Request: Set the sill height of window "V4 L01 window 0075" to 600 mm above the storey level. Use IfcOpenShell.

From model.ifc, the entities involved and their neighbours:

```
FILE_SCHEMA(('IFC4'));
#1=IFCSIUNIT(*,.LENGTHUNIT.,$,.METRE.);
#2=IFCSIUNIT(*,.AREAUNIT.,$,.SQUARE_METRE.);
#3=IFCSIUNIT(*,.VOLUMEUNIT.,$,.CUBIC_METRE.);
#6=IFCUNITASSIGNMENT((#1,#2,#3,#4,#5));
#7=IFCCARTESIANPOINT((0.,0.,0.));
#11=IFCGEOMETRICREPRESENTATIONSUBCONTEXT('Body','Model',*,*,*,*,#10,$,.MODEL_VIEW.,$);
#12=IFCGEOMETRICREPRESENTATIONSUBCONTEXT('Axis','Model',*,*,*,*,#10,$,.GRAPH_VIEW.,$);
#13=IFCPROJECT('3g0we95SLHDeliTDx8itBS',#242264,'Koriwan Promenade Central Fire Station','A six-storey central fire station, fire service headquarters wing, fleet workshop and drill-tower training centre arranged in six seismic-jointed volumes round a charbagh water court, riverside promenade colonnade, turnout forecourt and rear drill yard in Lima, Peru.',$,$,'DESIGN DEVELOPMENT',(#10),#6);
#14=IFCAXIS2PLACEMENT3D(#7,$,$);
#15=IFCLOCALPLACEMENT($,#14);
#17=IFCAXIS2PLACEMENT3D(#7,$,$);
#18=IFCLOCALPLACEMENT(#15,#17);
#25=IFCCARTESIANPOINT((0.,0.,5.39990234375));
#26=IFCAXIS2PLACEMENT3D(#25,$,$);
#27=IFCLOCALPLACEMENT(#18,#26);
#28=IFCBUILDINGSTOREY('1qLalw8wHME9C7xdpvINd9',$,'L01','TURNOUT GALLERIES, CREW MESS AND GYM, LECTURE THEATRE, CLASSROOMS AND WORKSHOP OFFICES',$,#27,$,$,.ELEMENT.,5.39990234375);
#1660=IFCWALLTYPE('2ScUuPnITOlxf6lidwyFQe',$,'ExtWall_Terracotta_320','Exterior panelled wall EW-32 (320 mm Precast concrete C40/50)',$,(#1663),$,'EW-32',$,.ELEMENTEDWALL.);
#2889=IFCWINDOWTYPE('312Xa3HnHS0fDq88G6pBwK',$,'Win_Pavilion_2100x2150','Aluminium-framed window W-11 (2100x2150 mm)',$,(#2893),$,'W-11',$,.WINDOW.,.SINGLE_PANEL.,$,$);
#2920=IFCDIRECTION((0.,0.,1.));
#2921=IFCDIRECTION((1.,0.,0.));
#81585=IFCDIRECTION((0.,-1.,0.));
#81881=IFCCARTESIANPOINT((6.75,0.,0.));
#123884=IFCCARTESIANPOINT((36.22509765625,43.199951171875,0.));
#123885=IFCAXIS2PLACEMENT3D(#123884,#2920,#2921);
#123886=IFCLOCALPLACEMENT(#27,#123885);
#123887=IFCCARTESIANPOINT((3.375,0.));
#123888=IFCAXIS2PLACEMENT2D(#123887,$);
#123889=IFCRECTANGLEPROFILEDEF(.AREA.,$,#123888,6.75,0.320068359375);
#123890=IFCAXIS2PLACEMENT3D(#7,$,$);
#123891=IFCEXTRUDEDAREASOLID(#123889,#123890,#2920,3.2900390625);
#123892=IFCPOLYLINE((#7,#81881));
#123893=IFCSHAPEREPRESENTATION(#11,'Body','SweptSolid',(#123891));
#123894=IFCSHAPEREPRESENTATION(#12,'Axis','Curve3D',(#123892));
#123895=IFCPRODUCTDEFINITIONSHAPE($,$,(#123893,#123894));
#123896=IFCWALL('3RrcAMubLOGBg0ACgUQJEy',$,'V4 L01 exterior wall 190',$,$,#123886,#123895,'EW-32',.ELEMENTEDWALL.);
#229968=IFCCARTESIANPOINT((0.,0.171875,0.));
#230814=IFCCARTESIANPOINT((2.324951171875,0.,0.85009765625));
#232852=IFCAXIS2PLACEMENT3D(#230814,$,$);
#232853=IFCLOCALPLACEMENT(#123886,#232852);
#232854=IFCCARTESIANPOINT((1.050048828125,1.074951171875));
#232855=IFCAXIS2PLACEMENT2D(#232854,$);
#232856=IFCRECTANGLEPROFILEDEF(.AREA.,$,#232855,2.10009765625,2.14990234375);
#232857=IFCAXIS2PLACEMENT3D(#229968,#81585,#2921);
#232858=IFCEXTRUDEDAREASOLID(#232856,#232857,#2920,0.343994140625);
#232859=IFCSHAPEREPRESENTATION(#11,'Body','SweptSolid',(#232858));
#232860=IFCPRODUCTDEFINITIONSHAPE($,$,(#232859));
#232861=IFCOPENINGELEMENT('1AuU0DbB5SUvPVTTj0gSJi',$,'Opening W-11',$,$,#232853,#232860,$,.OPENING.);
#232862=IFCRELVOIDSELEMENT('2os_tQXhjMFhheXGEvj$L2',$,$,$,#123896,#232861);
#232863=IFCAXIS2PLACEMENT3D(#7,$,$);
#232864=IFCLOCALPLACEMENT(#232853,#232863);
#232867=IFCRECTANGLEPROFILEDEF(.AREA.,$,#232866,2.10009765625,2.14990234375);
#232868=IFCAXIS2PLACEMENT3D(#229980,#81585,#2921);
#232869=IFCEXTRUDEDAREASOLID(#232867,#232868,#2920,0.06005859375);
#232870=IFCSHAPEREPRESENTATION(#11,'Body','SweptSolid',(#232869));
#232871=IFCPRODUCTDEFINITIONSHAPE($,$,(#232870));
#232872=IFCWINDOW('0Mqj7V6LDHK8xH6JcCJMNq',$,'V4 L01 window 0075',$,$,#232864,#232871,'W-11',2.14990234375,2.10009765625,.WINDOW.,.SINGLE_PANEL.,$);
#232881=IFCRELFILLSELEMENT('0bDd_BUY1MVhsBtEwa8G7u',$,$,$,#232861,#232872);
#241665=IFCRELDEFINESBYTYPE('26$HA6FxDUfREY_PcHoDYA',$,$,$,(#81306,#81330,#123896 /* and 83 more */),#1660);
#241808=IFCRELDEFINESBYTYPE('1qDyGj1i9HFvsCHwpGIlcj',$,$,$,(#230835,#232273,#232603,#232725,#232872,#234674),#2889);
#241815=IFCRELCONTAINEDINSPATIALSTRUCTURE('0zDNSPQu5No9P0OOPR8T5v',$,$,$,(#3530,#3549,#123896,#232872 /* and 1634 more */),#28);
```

```python
import numpy as np
import ifcopenshell
import ifcopenshell.api.geometry
import ifcopenshell.geom
import ifcopenshell.util.element
import ifcopenshell.util.placement
import ifcopenshell.util.shape
import ifcopenshell.util.unit

model = ifcopenshell.open("model.ifc")
unit_scale = ifcopenshell.util.unit.calculate_unit_scale(model)

window = model.by_guid("0Mqj7V6LDHK8xH6JcCJMNq")
opening = window.FillsVoids[0].RelatingOpeningElement
storey = ifcopenshell.util.element.get_container(window, ifc_class="IfcBuildingStorey")
level = ifcopenshell.util.placement.get_local_placement(storey.ObjectPlacement)[2, 3]

# The opening's origin need not be at the sill, so measure its lowest point.
shape = ifcopenshell.geom.create_shape(ifcopenshell.geom.settings(), opening)
bottom = ifcopenshell.util.shape.get_shape_bottom_elevation(shape, shape.geometry) / unit_scale
dz = level + 0.6 - bottom

shift = np.array([0.0, 0.0, dz])
# The window is placed relative to its opening, so it follows when the opening moves.
matrix = ifcopenshell.util.placement.get_local_placement(opening.ObjectPlacement)
matrix[:3, 3] += shift
ifcopenshell.api.geometry.edit_object_placement(
    model, product=opening, matrix=matrix, is_si=False, should_transform_children=True
)

print(f"moved by {dz * unit_scale:+.3f} m")

model.write("model_rev.ifc")
```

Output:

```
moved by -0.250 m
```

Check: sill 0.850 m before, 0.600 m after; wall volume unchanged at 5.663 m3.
